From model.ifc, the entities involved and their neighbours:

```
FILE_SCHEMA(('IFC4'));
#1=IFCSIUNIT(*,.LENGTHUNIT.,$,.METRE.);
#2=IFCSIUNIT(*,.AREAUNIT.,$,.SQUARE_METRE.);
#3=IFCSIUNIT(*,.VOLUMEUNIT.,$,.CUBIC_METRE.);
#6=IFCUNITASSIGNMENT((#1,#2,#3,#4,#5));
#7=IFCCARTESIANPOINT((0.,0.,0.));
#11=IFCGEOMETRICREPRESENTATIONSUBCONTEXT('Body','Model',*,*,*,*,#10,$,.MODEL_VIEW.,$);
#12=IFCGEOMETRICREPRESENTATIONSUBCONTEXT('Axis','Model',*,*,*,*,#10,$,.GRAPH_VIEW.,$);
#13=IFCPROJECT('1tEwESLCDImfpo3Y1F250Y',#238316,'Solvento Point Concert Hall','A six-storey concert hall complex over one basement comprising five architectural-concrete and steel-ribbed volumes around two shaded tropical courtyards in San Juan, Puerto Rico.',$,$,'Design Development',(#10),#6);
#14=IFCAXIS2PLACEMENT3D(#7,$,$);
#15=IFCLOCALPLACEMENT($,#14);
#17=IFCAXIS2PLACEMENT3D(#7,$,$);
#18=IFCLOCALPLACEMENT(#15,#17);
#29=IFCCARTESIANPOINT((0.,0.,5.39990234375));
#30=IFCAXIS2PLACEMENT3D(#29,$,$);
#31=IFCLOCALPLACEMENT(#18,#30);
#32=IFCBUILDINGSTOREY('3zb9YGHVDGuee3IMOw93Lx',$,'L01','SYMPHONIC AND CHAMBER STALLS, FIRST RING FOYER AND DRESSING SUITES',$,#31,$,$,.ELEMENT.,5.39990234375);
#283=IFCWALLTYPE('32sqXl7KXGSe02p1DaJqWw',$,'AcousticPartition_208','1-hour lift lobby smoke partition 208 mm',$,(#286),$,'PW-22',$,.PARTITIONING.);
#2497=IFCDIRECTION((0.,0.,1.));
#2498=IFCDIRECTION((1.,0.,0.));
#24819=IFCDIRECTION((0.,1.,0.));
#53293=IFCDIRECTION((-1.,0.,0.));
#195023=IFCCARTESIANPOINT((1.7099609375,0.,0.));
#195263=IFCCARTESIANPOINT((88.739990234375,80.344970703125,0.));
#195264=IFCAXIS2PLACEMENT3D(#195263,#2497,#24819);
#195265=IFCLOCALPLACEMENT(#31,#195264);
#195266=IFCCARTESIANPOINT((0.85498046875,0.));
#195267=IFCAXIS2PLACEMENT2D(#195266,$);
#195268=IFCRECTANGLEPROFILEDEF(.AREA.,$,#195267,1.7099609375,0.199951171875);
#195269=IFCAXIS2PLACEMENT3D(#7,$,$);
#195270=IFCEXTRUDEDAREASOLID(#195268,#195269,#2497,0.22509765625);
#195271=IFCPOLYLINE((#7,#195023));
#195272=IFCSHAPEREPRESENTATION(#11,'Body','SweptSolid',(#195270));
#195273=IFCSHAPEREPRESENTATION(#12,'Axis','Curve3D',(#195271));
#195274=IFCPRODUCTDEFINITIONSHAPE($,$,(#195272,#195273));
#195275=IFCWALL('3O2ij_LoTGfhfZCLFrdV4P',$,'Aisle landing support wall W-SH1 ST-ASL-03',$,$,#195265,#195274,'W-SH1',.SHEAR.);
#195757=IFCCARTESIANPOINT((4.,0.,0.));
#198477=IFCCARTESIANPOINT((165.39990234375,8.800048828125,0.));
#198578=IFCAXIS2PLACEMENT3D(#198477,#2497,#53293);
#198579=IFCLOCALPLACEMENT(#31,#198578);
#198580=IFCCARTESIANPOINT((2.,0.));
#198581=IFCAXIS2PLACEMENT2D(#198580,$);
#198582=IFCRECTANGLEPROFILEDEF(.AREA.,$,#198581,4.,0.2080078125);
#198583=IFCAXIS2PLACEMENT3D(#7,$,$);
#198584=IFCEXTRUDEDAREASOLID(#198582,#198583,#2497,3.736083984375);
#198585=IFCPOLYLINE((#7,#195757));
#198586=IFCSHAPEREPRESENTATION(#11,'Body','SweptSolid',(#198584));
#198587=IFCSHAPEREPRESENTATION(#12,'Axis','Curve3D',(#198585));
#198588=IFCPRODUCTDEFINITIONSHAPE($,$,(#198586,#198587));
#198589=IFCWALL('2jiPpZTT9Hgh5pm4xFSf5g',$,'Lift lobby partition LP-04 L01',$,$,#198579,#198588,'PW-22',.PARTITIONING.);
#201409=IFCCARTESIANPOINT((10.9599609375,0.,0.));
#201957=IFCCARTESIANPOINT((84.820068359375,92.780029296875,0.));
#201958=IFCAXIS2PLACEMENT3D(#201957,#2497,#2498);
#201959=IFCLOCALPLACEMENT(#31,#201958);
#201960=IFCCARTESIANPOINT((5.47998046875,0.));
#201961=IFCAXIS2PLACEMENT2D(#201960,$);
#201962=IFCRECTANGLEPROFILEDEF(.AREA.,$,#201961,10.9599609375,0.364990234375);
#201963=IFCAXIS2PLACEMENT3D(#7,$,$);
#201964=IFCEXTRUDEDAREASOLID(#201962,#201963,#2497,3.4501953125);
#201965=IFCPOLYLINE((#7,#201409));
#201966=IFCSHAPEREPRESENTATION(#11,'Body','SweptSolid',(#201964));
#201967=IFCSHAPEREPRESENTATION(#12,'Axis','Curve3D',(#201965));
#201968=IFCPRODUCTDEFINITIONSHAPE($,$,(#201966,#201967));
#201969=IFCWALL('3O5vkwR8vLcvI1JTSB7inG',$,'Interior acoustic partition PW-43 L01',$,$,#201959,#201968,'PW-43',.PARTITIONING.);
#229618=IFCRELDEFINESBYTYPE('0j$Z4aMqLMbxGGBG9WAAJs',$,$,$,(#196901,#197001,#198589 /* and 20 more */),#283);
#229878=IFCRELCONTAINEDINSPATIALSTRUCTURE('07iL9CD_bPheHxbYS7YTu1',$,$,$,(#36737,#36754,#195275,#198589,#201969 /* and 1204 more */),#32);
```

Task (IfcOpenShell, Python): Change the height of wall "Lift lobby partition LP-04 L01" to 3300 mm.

```python
import ifcopenshell
import ifcopenshell.geom
import ifcopenshell.util.representation
import ifcopenshell.util.shape
import ifcopenshell.util.unit

model = ifcopenshell.open("model.ifc")
unit_scale = ifcopenshell.util.unit.calculate_unit_scale(model)
settings = ifcopenshell.geom.settings()


def volume(element):
    """Net volume in cubic metres, openings subtracted."""
    shape = ifcopenshell.geom.create_shape(settings, element)
    return ifcopenshell.util.shape.get_volume(shape.geometry)


wall = model.by_guid("2jiPpZTT9Hgh5pm4xFSf5g")
before = volume(wall)

body = ifcopenshell.util.representation.get_representation(wall, "Model", "Body")
solid = body.Items[0]
old_height = solid.Depth
solid.Depth = 3.3 / unit_scale
after = volume(wall)

print(f"height {old_height:g} -> {solid.Depth:g}, volume {before:.3f} -> {after:.3f} m3")

model.write("model_rev.ifc")
```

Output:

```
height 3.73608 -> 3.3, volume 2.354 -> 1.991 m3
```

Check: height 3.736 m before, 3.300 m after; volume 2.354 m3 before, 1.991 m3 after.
